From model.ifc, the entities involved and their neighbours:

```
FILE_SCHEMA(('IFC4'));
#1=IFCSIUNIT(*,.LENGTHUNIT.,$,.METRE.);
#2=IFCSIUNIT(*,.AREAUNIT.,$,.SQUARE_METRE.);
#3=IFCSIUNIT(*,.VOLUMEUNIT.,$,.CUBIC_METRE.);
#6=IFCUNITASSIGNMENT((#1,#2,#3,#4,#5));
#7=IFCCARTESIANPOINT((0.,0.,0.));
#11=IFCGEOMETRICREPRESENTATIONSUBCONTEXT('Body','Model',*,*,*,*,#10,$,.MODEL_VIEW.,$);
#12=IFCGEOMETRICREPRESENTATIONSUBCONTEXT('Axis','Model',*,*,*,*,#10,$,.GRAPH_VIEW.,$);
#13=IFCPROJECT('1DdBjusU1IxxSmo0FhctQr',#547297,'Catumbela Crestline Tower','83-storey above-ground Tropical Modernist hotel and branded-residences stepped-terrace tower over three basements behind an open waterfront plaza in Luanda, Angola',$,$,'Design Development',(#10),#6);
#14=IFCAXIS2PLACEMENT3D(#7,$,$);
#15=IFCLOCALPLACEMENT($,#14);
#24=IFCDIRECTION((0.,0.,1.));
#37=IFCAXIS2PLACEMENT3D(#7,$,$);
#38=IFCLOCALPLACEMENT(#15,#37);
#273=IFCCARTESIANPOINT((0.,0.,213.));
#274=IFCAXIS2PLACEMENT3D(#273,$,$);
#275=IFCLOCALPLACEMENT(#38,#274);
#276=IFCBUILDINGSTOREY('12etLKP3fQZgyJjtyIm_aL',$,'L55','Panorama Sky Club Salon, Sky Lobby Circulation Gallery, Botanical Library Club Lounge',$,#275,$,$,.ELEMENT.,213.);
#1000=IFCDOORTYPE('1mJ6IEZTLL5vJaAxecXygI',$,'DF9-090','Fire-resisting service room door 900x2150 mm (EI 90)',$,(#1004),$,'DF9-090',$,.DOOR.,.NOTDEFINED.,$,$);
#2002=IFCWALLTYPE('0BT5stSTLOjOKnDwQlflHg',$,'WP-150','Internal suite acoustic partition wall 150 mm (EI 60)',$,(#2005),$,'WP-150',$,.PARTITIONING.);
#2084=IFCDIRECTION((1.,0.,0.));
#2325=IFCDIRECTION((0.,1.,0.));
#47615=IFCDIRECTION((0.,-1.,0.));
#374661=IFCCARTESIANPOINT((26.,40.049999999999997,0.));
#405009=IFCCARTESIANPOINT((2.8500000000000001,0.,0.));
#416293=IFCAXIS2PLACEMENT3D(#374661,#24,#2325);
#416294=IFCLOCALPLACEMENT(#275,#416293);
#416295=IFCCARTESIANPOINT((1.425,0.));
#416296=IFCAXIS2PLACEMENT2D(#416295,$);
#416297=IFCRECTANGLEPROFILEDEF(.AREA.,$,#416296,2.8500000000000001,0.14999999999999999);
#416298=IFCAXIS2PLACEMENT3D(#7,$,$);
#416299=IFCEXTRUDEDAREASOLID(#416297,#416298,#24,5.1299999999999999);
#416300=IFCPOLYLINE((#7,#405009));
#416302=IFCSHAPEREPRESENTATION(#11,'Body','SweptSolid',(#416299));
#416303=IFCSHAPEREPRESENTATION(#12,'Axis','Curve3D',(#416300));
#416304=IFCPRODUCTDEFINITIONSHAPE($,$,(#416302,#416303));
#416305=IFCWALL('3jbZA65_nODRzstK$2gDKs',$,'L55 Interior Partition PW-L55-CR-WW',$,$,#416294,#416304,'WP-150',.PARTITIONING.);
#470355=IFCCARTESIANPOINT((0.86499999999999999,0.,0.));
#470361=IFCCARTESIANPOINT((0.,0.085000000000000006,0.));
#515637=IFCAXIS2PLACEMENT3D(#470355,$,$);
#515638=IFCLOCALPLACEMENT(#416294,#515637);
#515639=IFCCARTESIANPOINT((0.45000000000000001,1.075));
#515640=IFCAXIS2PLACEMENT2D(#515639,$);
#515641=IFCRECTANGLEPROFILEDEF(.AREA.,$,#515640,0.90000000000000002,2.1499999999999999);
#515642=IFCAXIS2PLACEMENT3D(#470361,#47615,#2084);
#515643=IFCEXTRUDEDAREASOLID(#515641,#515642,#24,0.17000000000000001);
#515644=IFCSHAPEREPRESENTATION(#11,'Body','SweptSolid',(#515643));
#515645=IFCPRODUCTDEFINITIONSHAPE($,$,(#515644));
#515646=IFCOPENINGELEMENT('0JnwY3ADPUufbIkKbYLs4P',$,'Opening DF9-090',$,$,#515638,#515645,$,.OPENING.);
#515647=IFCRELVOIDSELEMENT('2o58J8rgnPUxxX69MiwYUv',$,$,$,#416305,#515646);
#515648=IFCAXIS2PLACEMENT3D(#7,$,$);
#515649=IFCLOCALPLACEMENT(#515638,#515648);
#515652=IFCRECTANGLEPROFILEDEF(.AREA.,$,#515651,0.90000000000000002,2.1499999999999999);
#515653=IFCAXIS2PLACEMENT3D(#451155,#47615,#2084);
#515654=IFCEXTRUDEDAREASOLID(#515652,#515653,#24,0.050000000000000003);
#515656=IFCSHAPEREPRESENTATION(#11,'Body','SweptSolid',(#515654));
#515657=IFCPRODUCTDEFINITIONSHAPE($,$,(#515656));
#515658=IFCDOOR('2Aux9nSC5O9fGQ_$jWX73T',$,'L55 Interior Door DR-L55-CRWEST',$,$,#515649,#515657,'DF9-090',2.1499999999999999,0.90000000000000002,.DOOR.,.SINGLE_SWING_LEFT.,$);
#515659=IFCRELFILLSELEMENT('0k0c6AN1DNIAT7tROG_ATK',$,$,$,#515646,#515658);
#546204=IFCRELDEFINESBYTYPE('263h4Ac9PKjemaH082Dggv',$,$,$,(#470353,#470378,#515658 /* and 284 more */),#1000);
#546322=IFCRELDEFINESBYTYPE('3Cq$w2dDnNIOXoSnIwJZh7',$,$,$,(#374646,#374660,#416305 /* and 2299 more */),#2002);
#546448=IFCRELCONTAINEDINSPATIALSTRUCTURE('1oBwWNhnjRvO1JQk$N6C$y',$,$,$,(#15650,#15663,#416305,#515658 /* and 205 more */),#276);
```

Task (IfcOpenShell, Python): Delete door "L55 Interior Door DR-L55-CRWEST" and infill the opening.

```python
import ifcopenshell
import ifcopenshell.api.feature
import ifcopenshell.api.root
import ifcopenshell.geom
import ifcopenshell.util.shape

model = ifcopenshell.open("model.ifc")
settings = ifcopenshell.geom.settings()


def volume(element):
    """Net volume in cubic metres, openings subtracted."""
    shape = ifcopenshell.geom.create_shape(settings, element)
    return ifcopenshell.util.shape.get_volume(shape.geometry)


door = model.by_guid("2Aux9nSC5O9fGQ_$jWX73T")
opening = door.FillsVoids[0].RelatingOpeningElement
wall = opening.VoidsElements[0].RelatingBuildingElement
before = volume(wall)

ifcopenshell.api.root.remove_product(model, product=door)
ifcopenshell.api.feature.remove_feature(model, feature=opening)

after = volume(wall)

print(f"wall volume {before:.3f} -> {after:.3f} m3")

model.write("model_updated.ifc")
```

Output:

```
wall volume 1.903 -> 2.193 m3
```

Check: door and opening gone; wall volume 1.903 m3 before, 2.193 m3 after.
